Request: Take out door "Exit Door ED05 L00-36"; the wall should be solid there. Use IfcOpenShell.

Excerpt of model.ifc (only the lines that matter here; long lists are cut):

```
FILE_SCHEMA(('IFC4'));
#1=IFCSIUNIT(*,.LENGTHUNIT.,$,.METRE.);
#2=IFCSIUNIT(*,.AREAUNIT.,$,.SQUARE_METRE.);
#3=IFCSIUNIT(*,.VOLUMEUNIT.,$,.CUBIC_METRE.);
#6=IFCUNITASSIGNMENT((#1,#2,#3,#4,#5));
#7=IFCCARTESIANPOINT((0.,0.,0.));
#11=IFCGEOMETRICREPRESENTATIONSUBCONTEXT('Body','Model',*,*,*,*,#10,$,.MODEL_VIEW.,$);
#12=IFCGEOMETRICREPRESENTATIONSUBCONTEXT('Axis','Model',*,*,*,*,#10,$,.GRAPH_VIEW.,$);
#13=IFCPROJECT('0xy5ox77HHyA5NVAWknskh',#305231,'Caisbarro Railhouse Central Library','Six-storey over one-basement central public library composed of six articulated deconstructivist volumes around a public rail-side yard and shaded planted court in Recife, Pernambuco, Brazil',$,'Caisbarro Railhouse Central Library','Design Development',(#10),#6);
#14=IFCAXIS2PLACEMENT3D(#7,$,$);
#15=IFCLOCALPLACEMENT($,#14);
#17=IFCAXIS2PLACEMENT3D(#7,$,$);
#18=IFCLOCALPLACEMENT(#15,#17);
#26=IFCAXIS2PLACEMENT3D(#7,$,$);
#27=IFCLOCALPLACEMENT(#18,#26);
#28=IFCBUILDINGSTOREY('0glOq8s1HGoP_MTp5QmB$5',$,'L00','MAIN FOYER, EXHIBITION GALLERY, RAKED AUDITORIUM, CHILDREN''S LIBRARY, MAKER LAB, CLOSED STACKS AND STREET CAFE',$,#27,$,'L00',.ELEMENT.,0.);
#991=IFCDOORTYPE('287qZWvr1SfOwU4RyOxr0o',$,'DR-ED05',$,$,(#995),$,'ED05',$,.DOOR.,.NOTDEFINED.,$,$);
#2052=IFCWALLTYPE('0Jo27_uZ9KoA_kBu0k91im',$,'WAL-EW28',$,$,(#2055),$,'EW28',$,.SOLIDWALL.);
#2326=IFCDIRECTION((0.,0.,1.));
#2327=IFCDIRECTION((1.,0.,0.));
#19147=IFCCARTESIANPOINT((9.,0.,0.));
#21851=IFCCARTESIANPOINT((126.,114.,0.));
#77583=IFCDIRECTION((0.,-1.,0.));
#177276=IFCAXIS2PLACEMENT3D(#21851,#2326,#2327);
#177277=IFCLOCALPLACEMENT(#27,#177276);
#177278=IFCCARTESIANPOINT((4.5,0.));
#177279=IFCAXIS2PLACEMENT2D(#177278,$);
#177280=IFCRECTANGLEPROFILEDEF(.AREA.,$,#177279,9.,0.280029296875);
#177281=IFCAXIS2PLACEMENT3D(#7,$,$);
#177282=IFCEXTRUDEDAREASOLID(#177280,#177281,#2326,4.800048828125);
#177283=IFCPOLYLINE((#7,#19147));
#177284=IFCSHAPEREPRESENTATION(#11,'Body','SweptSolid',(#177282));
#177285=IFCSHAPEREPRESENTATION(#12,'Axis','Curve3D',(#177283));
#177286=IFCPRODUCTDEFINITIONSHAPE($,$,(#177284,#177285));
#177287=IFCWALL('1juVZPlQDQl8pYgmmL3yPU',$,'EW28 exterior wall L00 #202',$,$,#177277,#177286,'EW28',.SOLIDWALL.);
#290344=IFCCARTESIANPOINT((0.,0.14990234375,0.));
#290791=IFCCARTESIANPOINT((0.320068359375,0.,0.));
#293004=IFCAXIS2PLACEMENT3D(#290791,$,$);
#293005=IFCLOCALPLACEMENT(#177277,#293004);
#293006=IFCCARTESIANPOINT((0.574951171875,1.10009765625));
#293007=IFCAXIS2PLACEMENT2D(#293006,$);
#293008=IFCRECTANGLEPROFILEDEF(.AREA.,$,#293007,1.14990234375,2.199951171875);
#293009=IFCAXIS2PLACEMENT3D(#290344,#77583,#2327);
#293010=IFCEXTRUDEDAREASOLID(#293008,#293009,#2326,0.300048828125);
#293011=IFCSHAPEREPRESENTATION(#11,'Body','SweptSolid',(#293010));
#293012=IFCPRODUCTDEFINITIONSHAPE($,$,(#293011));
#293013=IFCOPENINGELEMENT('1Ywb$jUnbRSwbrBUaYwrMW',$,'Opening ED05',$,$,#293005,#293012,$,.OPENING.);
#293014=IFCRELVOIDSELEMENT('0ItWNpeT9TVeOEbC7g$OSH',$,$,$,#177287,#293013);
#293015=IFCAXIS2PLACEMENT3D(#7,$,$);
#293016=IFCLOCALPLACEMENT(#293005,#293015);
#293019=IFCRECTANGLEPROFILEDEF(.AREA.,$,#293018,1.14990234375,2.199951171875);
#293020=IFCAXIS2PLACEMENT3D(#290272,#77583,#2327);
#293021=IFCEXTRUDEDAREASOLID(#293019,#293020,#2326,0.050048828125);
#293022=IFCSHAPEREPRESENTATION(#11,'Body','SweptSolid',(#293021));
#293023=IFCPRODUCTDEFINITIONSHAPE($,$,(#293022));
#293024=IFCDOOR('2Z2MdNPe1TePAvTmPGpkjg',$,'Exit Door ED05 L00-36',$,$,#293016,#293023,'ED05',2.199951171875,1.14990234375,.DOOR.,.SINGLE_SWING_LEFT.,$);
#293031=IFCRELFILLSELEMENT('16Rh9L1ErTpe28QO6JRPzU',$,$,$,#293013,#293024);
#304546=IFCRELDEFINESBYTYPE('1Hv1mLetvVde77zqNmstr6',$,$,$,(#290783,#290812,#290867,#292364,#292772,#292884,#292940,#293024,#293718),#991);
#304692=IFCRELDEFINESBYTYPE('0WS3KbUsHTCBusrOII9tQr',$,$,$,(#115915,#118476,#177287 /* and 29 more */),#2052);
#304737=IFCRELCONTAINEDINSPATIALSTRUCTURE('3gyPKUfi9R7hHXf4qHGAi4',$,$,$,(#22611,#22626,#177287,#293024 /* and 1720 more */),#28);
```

```python
import ifcopenshell
import ifcopenshell.api.feature
import ifcopenshell.api.root
import ifcopenshell.geom
import ifcopenshell.util.shape

model = ifcopenshell.open("model.ifc")
settings = ifcopenshell.geom.settings()


def volume(element):
    """Net volume in cubic metres, openings subtracted."""
    shape = ifcopenshell.geom.create_shape(settings, element)
    return ifcopenshell.util.shape.get_volume(shape.geometry)


door = model.by_guid("2Z2MdNPe1TePAvTmPGpkjg")
opening = door.FillsVoids[0].RelatingOpeningElement
wall = opening.VoidsElements[0].RelatingBuildingElement
before = volume(wall)

ifcopenshell.api.root.remove_product(model, product=door)
ifcopenshell.api.feature.remove_feature(model, feature=opening)

after = volume(wall)

print(f"wall volume {before:.3f} -> {after:.3f} m3")

model.write("model-out.ifc")
```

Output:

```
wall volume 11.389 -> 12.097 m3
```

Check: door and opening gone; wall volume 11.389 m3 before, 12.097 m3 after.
